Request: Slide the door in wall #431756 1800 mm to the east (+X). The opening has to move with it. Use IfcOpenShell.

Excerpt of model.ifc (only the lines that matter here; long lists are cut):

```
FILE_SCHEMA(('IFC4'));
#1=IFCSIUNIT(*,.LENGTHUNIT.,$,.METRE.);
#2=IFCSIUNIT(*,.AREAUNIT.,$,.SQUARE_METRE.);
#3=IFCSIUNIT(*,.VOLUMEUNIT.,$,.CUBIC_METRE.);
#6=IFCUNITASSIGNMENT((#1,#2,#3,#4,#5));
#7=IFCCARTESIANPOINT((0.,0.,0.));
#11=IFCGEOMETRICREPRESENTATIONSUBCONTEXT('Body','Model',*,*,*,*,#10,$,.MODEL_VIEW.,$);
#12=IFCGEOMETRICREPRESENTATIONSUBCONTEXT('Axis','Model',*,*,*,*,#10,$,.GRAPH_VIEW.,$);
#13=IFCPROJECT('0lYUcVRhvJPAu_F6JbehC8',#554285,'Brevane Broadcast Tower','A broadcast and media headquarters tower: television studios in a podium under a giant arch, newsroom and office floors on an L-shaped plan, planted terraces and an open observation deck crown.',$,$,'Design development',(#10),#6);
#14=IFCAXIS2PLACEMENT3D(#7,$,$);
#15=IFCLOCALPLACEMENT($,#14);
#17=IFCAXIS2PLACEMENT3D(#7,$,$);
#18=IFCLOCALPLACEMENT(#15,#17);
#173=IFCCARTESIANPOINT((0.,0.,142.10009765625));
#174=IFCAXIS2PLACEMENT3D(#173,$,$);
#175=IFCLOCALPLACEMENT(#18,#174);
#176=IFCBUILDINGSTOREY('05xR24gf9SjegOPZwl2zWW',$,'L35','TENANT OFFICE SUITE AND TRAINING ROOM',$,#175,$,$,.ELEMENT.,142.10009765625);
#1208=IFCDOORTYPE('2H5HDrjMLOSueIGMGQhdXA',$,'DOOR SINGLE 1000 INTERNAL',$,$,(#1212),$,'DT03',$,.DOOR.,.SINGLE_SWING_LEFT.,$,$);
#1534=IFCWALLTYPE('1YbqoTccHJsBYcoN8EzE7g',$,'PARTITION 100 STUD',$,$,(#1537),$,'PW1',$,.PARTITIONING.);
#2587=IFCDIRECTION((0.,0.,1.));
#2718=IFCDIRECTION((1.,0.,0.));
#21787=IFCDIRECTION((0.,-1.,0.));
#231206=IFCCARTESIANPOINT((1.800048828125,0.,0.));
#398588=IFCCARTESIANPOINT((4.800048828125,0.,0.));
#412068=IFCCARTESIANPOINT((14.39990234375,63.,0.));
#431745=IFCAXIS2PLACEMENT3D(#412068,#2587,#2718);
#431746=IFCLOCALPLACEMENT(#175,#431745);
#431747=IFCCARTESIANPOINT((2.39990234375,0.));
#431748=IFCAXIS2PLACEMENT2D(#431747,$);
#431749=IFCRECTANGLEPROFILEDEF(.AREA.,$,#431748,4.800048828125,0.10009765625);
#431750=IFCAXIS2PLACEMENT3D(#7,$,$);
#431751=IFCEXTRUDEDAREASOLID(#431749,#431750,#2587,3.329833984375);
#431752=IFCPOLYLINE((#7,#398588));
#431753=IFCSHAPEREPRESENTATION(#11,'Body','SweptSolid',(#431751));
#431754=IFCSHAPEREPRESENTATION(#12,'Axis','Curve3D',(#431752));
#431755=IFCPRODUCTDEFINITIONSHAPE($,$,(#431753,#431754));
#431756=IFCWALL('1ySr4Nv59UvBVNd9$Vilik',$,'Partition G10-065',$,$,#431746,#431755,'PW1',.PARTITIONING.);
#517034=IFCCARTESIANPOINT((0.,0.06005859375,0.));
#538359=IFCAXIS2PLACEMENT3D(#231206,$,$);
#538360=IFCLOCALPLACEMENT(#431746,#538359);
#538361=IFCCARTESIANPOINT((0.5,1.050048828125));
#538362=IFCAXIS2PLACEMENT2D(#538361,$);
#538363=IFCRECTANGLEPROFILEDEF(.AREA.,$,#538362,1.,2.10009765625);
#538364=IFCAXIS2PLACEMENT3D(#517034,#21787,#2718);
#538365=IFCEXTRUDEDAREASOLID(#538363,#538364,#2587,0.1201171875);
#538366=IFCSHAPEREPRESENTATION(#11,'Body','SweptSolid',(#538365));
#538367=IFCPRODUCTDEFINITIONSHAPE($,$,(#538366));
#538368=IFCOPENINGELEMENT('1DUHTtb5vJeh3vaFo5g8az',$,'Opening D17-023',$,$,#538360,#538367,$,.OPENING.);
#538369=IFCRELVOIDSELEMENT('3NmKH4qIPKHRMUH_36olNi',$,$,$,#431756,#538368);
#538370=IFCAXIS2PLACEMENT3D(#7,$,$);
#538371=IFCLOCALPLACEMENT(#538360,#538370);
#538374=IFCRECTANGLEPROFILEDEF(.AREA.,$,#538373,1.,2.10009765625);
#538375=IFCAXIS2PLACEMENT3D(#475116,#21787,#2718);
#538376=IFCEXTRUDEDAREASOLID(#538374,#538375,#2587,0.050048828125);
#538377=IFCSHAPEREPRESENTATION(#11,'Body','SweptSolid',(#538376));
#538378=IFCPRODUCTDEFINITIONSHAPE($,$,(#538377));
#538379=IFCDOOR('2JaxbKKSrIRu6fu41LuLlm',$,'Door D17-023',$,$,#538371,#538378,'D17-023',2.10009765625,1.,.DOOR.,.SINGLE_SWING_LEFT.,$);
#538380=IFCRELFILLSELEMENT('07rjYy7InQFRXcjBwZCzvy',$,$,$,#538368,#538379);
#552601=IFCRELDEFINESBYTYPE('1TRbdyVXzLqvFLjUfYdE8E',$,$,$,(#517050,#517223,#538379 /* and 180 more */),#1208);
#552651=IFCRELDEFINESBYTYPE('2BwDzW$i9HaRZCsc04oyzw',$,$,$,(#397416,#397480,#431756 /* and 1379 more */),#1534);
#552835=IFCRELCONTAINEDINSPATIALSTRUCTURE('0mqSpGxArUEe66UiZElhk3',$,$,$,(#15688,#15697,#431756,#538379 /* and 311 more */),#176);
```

```python
import ifcopenshell
import ifcopenshell.api.geometry
import ifcopenshell.util.placement

model = ifcopenshell.open("model.ifc")

door = model.by_guid("2JaxbKKSrIRu6fu41LuLlm")
opening = door.FillsVoids[0].RelatingOpeningElement
wall = opening.VoidsElements[0].RelatingBuildingElement

wall_matrix = ifcopenshell.util.placement.get_local_placement(wall.ObjectPlacement)
shift = wall_matrix[:3, 0] * 1.8
before = ifcopenshell.util.placement.get_local_placement(door.ObjectPlacement)[:3, 3].copy()

# The door is placed relative to its opening, so it follows when the opening moves.
matrix = ifcopenshell.util.placement.get_local_placement(opening.ObjectPlacement)
matrix[:3, 3] += shift
ifcopenshell.api.geometry.edit_object_placement(
    model, product=opening, matrix=matrix, is_si=False, should_transform_children=True
)

after = ifcopenshell.util.placement.get_local_placement(door.ObjectPlacement)[:3, 3]
print("door moved by", (after - before).round(3) + 0.0)

model.write("model_edited.ifc")
```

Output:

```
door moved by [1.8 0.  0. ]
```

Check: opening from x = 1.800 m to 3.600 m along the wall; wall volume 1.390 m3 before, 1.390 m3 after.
